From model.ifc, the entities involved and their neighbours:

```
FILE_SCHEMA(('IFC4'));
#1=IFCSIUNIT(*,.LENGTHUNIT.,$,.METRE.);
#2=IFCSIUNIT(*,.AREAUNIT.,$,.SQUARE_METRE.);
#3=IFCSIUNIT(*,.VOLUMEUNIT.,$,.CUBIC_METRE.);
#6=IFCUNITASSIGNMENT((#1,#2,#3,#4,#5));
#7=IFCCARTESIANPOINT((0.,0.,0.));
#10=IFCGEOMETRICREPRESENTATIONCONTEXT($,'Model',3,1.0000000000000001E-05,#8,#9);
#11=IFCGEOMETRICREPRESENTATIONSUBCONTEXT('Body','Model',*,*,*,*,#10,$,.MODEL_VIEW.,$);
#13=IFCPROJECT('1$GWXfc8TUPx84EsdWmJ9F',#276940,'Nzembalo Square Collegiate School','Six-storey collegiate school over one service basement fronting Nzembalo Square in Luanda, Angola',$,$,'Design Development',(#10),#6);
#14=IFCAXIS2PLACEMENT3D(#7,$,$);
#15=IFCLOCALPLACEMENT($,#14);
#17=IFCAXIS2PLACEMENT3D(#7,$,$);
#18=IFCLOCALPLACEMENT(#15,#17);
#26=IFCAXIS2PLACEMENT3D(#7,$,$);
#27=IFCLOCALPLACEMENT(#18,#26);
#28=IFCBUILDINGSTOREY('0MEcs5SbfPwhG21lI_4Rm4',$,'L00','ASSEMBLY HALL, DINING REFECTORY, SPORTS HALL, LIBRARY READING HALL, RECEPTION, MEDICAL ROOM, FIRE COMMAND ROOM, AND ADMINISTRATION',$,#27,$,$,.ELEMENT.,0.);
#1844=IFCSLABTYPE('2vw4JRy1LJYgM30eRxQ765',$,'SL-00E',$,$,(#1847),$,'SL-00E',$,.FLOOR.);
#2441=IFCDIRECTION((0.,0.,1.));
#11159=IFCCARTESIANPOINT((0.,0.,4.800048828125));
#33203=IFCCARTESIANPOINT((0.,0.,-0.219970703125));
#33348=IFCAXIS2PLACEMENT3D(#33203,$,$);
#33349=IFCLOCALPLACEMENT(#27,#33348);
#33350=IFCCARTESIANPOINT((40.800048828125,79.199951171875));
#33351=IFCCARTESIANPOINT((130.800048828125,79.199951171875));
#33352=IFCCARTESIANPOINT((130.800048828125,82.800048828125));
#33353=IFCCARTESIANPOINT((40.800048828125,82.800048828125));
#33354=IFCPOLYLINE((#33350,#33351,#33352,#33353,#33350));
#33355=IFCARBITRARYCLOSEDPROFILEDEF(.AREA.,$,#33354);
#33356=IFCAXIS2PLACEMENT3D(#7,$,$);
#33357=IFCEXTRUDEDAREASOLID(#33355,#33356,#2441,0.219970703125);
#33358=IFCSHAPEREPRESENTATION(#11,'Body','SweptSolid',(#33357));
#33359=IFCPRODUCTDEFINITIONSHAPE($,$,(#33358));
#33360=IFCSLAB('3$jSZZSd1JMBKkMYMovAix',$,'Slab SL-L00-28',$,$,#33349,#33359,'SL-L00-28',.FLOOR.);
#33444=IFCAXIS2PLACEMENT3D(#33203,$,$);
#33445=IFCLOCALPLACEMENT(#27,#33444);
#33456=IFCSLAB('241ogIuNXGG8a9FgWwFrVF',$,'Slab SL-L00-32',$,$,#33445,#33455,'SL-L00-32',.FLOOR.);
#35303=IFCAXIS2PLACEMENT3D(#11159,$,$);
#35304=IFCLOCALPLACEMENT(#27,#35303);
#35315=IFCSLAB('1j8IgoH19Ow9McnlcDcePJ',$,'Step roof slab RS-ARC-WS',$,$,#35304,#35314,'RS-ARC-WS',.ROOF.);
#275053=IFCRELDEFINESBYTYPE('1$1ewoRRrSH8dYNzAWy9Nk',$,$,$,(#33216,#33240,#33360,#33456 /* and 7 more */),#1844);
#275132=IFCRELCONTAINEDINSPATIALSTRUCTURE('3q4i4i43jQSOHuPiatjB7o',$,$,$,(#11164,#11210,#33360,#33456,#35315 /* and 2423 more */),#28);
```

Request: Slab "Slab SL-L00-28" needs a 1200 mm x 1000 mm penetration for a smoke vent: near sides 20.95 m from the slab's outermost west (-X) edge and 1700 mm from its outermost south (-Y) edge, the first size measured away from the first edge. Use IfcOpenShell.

```python
import numpy as np
import ifcopenshell
import ifcopenshell.api.feature
import ifcopenshell.api.geometry
import ifcopenshell.api.root
import ifcopenshell.geom
import ifcopenshell.util.placement
import ifcopenshell.util.representation
import ifcopenshell.util.shape
import ifcopenshell.util.unit

model = ifcopenshell.open("model.ifc")
unit_scale = ifcopenshell.util.unit.calculate_unit_scale(model)
settings = ifcopenshell.geom.settings()


def volume(element):
    """Net volume in cubic metres, openings subtracted."""
    shape = ifcopenshell.geom.create_shape(settings, element)
    return ifcopenshell.util.shape.get_volume(shape.geometry)


slab = model.by_id(33360)
before = volume(slab)

# Extent in the slab's own axes, in metres. The edges named are its -X and -Y sides.
slab_shape = ifcopenshell.geom.create_shape(settings, slab)
vertices = ifcopenshell.util.shape.get_vertices(slab_shape.geometry)
x_min, y_min, bottom = vertices.min(axis=0)
top = vertices[:, 2].max()

opening = ifcopenshell.api.root.create_entity(model, ifc_class="IfcOpeningElement", name="Smoke vent opening", predefined_type="OPENING")
context = ifcopenshell.util.representation.get_context(model, "Model", "Body", "MODEL_VIEW")
width, depth = 1.2, 1
outline = [(0.0, 0.0), (width, 0.0), (width, depth), (0.0, depth), (0.0, 0.0)]
# Overshoot both faces by 50 mm so the cut is clean.
shape = ifcopenshell.api.geometry.add_slab_representation(
    model, context=context, depth=top - bottom + 0.1, polyline=outline
)
ifcopenshell.api.geometry.assign_representation(model, product=opening, representation=shape)

matrix = ifcopenshell.util.placement.get_local_placement(slab.ObjectPlacement)
matrix[:, 3] = matrix @ np.append(np.array([x_min + 20.95, y_min + 1.7, bottom - 0.05]) / unit_scale, 1.0)
ifcopenshell.api.geometry.edit_object_placement(model, product=opening, matrix=matrix, is_si=False)
ifcopenshell.api.feature.add_feature(model, feature=opening, element=slab)

after = volume(slab)

print(f"slab volume {before:.3f} -> {after:.3f} m3")

model.write("model_v2.ifc")
```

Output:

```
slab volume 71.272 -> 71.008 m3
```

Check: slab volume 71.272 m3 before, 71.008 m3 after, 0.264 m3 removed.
